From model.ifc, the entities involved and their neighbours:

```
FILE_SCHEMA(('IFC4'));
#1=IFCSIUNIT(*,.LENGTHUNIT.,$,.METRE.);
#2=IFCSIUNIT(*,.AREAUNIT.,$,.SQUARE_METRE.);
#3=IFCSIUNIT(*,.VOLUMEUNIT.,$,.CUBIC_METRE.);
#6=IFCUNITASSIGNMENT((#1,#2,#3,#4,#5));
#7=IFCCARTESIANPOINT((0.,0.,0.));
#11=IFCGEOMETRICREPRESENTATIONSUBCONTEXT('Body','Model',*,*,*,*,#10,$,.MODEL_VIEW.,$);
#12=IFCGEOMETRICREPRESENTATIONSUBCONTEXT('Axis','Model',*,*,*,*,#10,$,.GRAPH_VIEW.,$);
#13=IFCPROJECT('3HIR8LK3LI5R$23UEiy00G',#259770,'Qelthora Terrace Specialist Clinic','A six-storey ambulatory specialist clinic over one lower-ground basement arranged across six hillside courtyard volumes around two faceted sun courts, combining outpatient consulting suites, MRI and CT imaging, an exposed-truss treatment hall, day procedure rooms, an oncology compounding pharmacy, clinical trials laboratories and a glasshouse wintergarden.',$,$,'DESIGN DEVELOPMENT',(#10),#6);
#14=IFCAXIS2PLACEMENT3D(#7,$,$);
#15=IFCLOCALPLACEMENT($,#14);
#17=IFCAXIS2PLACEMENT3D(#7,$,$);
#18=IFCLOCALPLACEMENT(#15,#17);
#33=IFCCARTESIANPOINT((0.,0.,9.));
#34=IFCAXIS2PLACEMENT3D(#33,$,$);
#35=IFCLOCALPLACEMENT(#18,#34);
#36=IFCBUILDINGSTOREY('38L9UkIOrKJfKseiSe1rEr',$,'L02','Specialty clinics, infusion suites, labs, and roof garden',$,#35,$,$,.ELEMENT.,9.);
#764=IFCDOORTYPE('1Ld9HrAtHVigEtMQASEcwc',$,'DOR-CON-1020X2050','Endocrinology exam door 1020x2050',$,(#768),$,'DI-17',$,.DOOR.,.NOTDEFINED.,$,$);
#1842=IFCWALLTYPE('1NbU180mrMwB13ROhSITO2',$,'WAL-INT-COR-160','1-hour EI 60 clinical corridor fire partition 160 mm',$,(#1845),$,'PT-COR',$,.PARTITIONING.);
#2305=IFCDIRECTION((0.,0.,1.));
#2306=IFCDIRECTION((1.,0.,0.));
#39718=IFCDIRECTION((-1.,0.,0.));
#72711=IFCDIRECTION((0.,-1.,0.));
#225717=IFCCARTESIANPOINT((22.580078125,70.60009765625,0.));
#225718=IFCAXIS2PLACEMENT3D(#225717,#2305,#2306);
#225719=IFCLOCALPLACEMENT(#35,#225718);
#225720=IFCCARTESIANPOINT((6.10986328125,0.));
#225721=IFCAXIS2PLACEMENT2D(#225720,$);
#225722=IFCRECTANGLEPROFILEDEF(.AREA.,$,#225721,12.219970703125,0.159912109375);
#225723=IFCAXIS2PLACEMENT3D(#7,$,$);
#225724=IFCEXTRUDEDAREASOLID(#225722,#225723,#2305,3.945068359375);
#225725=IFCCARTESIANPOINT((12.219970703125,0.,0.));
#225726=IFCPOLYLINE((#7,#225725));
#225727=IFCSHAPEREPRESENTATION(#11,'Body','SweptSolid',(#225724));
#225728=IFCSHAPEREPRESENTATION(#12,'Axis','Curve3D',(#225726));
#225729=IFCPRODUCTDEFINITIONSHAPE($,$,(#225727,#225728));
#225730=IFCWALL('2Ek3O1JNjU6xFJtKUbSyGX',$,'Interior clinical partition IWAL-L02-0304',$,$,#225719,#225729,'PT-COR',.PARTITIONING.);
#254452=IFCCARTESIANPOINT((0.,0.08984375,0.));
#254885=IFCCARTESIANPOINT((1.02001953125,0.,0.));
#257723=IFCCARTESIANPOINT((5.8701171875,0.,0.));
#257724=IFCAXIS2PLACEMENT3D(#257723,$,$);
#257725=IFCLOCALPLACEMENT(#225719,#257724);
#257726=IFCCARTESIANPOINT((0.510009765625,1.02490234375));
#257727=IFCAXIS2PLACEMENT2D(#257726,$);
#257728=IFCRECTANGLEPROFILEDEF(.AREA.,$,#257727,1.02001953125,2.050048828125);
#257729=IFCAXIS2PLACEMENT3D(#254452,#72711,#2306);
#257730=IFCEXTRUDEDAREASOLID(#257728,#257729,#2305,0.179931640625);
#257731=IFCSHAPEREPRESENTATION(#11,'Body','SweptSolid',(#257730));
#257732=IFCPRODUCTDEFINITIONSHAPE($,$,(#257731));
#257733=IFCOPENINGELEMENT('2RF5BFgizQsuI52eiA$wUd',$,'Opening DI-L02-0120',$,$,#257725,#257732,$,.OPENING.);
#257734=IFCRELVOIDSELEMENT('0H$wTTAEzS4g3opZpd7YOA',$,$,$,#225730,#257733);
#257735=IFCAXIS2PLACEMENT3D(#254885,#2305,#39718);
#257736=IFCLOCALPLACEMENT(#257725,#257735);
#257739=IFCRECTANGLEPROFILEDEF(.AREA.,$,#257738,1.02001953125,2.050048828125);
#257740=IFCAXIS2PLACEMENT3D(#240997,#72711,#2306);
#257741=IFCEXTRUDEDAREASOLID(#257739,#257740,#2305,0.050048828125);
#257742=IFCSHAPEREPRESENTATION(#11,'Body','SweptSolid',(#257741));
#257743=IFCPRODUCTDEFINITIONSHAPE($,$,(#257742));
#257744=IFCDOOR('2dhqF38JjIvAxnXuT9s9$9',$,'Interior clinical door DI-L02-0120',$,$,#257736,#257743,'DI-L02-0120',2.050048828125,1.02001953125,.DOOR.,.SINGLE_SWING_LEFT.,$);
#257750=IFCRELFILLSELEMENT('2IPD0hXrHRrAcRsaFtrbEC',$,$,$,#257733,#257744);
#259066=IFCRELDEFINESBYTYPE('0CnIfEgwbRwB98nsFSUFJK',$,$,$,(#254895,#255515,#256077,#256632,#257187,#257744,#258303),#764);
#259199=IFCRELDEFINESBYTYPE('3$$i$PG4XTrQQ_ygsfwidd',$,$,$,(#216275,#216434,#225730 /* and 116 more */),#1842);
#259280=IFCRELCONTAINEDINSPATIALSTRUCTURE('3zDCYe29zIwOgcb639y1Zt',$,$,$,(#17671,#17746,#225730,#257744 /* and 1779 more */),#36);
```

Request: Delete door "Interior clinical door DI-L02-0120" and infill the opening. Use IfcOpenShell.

```python
import ifcopenshell
import ifcopenshell.api.feature
import ifcopenshell.api.root
import ifcopenshell.geom
import ifcopenshell.util.shape

model = ifcopenshell.open("model.ifc")
settings = ifcopenshell.geom.settings()


def volume(element):
    """Net volume in cubic metres, openings subtracted."""
    shape = ifcopenshell.geom.create_shape(settings, element)
    return ifcopenshell.util.shape.get_volume(shape.geometry)


door = model.by_guid("2dhqF38JjIvAxnXuT9s9$9")
opening = door.FillsVoids[0].RelatingOpeningElement
wall = opening.VoidsElements[0].RelatingBuildingElement
before = volume(wall)

ifcopenshell.api.root.remove_product(model, product=door)
ifcopenshell.api.feature.remove_feature(model, feature=opening)

after = volume(wall)

print(f"wall volume {before:.3f} -> {after:.3f} m3")

model.write("model_rev.ifc")
```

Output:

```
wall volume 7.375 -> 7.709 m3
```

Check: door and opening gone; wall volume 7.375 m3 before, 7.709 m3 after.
